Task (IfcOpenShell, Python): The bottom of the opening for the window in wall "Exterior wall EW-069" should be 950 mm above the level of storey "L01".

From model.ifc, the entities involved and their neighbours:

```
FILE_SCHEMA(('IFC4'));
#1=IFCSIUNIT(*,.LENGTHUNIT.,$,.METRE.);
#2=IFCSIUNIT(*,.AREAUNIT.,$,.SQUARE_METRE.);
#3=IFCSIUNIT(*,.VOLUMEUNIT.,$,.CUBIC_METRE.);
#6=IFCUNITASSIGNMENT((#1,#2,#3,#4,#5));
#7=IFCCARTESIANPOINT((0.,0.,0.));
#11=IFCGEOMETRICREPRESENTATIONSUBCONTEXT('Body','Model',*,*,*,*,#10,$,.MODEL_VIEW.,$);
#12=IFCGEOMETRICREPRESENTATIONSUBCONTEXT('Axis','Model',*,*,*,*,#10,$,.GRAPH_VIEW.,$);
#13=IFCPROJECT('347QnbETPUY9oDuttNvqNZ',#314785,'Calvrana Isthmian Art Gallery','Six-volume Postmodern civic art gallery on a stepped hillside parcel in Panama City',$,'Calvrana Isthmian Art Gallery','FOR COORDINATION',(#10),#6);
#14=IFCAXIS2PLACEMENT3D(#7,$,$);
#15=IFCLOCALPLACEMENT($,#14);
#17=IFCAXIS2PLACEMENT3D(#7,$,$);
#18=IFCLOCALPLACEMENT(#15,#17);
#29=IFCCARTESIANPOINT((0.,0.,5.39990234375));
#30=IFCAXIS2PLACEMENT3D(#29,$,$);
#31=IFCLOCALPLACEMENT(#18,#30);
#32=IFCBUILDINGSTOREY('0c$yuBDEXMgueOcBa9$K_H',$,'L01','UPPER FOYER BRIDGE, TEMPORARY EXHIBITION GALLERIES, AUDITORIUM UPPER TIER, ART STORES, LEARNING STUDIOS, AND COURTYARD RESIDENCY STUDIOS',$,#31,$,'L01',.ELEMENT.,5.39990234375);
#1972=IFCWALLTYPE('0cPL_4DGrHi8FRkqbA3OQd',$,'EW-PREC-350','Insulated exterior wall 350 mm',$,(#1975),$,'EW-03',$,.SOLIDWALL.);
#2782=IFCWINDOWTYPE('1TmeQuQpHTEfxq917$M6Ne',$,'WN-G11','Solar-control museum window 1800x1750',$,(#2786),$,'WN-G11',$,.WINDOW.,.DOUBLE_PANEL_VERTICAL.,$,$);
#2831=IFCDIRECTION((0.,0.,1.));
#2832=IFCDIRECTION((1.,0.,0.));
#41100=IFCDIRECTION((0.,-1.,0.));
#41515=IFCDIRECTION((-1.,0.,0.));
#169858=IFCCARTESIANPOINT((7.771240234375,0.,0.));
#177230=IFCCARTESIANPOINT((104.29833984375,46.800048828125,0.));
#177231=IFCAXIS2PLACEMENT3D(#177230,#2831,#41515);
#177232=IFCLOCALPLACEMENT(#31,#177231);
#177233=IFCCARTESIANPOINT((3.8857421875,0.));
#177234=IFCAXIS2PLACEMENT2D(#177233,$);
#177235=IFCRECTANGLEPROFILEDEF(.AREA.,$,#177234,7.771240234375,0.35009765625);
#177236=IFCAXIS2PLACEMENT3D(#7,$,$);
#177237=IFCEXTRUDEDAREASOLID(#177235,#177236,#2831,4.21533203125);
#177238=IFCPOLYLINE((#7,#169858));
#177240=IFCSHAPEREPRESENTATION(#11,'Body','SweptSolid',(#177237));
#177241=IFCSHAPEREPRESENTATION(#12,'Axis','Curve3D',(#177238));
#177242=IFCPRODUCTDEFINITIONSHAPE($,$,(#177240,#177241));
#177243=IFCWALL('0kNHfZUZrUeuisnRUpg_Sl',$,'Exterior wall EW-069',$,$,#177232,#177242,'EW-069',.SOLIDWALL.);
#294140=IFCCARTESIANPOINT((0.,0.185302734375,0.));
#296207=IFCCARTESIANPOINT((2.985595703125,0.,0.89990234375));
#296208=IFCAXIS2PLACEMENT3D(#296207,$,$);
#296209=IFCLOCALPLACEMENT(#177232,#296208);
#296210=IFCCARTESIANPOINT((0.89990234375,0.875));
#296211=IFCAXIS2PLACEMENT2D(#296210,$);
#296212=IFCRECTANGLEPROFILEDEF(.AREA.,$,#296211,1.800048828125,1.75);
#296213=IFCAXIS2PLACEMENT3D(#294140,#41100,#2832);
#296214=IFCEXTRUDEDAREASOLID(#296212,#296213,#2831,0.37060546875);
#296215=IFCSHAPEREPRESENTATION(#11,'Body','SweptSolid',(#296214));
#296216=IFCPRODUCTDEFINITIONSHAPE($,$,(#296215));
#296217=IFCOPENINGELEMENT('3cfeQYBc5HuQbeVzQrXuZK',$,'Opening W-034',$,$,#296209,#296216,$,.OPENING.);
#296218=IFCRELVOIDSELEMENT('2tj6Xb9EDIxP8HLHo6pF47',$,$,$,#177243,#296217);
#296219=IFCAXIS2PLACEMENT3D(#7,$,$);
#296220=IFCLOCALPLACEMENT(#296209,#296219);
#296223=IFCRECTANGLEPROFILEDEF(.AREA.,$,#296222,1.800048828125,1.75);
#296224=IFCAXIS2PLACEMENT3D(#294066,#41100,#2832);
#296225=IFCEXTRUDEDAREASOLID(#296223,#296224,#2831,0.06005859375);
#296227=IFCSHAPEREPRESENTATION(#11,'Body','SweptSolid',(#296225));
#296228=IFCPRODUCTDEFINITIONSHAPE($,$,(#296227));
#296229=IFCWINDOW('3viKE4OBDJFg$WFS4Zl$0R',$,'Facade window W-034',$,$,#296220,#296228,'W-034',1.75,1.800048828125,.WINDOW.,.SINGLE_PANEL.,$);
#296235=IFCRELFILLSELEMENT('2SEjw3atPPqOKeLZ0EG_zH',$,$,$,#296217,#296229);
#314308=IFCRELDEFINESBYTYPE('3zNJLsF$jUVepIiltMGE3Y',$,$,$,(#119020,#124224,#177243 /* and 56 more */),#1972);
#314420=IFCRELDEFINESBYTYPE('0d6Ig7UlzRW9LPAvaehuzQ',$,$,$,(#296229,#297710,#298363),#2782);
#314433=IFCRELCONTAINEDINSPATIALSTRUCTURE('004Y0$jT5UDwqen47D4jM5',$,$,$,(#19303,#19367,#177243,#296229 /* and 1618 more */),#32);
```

```python
import numpy as np
import ifcopenshell
import ifcopenshell.api.geometry
import ifcopenshell.geom
import ifcopenshell.util.element
import ifcopenshell.util.placement
import ifcopenshell.util.shape
import ifcopenshell.util.unit

model = ifcopenshell.open("model.ifc")
unit_scale = ifcopenshell.util.unit.calculate_unit_scale(model)

window = model.by_guid("3viKE4OBDJFg$WFS4Zl$0R")
opening = window.FillsVoids[0].RelatingOpeningElement
storey = ifcopenshell.util.element.get_container(window, ifc_class="IfcBuildingStorey")
level = ifcopenshell.util.placement.get_local_placement(storey.ObjectPlacement)[2, 3]

# The opening's origin need not be at the sill, so measure its lowest point.
shape = ifcopenshell.geom.create_shape(ifcopenshell.geom.settings(), opening)
bottom = ifcopenshell.util.shape.get_shape_bottom_elevation(shape, shape.geometry) / unit_scale
dz = level + 0.95 / unit_scale - bottom

shift = np.array([0.0, 0.0, dz])
# The window is placed relative to its opening, so it follows when the opening moves.
matrix = ifcopenshell.util.placement.get_local_placement(opening.ObjectPlacement)
matrix[:3, 3] += shift
ifcopenshell.api.geometry.edit_object_placement(
    model, product=opening, matrix=matrix, is_si=False, should_transform_children=True
)

print(f"moved by {dz * unit_scale:+.3f} m")

model.write("model_edited.ifc")
```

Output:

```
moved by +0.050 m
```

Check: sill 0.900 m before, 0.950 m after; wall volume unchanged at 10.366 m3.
